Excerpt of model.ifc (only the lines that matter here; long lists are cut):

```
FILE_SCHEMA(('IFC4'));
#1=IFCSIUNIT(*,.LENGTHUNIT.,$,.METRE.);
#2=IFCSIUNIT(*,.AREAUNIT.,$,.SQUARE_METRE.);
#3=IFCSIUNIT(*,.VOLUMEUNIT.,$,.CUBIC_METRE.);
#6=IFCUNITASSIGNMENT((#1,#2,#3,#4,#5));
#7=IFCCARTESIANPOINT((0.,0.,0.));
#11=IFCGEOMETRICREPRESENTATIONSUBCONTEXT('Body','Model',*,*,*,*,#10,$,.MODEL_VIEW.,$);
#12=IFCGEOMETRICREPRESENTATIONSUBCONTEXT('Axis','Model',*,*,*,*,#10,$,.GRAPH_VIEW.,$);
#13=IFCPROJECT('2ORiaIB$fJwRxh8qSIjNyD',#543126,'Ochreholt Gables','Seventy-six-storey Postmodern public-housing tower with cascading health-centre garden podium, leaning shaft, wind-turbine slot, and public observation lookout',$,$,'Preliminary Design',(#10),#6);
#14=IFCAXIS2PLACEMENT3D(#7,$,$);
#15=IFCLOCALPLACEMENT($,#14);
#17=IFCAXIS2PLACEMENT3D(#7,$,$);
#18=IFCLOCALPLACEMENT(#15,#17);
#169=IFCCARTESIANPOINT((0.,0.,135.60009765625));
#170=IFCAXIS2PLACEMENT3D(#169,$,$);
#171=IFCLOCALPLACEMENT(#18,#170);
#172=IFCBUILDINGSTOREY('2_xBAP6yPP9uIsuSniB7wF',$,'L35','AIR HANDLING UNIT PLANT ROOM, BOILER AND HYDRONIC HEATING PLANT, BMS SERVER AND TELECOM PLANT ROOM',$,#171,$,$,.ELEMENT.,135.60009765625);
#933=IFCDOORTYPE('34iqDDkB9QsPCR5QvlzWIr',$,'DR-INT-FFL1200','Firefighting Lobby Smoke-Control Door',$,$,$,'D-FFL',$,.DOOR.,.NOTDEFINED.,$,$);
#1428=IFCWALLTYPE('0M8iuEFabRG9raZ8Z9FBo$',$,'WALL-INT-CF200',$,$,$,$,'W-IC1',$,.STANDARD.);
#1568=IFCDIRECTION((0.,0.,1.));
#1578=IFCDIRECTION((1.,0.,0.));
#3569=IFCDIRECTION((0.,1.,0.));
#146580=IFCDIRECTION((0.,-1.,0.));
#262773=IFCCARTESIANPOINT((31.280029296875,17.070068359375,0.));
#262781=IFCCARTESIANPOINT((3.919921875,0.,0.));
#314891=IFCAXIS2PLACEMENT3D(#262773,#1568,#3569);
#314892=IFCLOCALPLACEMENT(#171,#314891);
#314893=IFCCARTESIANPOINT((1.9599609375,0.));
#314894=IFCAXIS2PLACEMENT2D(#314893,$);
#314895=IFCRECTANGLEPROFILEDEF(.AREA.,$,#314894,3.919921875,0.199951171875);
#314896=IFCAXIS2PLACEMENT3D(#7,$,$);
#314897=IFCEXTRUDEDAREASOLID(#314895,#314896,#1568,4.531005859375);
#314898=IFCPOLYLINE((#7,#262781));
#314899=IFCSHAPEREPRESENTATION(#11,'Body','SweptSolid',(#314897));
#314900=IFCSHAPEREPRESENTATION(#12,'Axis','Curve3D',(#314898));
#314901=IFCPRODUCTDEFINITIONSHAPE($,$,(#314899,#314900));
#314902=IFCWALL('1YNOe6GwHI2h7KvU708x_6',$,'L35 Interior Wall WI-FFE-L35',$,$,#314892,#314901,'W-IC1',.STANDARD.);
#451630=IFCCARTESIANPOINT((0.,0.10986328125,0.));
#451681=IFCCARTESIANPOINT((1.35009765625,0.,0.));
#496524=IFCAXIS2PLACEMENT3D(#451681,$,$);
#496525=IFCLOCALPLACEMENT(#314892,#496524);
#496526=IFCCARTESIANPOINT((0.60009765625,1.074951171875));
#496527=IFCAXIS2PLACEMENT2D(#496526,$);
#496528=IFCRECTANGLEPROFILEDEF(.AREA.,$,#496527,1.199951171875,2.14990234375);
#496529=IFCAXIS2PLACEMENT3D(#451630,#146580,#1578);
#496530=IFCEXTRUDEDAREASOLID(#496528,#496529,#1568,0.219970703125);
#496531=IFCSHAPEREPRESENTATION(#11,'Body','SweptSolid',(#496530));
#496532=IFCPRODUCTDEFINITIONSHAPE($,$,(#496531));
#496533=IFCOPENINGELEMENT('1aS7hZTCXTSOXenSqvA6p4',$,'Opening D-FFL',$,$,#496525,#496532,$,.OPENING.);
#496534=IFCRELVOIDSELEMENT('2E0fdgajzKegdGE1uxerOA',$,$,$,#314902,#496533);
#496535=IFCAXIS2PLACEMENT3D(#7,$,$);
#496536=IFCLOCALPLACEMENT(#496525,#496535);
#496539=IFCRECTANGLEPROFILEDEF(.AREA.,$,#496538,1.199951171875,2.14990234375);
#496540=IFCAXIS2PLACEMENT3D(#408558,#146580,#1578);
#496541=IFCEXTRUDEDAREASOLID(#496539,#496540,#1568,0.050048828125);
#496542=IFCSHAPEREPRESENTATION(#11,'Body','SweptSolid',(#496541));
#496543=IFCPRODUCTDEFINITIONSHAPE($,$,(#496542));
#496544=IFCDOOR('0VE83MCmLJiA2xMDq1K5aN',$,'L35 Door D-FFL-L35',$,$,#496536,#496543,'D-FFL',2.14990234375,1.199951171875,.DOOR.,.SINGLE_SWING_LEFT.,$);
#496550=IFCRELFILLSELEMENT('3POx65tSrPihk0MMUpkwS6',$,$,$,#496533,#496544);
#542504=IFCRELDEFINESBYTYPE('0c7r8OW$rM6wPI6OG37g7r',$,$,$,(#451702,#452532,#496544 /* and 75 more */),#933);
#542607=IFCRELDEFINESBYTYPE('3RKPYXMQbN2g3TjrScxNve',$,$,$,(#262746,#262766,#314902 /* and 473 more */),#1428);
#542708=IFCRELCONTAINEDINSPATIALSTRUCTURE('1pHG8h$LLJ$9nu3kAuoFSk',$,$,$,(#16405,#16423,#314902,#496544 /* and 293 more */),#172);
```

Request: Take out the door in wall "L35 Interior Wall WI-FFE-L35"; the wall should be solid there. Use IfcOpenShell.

```python
import ifcopenshell
import ifcopenshell.api.feature
import ifcopenshell.api.root
import ifcopenshell.geom
import ifcopenshell.util.shape

model = ifcopenshell.open("model.ifc")
settings = ifcopenshell.geom.settings()


def volume(element):
    """Net volume in cubic metres, openings subtracted."""
    shape = ifcopenshell.geom.create_shape(settings, element)
    return ifcopenshell.util.shape.get_volume(shape.geometry)


door = model.by_guid("0VE83MCmLJiA2xMDq1K5aN")
opening = door.FillsVoids[0].RelatingOpeningElement
wall = opening.VoidsElements[0].RelatingBuildingElement
before = volume(wall)

ifcopenshell.api.root.remove_product(model, product=door)
ifcopenshell.api.feature.remove_feature(model, feature=opening)

after = volume(wall)

print(f"wall volume {before:.3f} -> {after:.3f} m3")

model.write("model_rev.ifc")
```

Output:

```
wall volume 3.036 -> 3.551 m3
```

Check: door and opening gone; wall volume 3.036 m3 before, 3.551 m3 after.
